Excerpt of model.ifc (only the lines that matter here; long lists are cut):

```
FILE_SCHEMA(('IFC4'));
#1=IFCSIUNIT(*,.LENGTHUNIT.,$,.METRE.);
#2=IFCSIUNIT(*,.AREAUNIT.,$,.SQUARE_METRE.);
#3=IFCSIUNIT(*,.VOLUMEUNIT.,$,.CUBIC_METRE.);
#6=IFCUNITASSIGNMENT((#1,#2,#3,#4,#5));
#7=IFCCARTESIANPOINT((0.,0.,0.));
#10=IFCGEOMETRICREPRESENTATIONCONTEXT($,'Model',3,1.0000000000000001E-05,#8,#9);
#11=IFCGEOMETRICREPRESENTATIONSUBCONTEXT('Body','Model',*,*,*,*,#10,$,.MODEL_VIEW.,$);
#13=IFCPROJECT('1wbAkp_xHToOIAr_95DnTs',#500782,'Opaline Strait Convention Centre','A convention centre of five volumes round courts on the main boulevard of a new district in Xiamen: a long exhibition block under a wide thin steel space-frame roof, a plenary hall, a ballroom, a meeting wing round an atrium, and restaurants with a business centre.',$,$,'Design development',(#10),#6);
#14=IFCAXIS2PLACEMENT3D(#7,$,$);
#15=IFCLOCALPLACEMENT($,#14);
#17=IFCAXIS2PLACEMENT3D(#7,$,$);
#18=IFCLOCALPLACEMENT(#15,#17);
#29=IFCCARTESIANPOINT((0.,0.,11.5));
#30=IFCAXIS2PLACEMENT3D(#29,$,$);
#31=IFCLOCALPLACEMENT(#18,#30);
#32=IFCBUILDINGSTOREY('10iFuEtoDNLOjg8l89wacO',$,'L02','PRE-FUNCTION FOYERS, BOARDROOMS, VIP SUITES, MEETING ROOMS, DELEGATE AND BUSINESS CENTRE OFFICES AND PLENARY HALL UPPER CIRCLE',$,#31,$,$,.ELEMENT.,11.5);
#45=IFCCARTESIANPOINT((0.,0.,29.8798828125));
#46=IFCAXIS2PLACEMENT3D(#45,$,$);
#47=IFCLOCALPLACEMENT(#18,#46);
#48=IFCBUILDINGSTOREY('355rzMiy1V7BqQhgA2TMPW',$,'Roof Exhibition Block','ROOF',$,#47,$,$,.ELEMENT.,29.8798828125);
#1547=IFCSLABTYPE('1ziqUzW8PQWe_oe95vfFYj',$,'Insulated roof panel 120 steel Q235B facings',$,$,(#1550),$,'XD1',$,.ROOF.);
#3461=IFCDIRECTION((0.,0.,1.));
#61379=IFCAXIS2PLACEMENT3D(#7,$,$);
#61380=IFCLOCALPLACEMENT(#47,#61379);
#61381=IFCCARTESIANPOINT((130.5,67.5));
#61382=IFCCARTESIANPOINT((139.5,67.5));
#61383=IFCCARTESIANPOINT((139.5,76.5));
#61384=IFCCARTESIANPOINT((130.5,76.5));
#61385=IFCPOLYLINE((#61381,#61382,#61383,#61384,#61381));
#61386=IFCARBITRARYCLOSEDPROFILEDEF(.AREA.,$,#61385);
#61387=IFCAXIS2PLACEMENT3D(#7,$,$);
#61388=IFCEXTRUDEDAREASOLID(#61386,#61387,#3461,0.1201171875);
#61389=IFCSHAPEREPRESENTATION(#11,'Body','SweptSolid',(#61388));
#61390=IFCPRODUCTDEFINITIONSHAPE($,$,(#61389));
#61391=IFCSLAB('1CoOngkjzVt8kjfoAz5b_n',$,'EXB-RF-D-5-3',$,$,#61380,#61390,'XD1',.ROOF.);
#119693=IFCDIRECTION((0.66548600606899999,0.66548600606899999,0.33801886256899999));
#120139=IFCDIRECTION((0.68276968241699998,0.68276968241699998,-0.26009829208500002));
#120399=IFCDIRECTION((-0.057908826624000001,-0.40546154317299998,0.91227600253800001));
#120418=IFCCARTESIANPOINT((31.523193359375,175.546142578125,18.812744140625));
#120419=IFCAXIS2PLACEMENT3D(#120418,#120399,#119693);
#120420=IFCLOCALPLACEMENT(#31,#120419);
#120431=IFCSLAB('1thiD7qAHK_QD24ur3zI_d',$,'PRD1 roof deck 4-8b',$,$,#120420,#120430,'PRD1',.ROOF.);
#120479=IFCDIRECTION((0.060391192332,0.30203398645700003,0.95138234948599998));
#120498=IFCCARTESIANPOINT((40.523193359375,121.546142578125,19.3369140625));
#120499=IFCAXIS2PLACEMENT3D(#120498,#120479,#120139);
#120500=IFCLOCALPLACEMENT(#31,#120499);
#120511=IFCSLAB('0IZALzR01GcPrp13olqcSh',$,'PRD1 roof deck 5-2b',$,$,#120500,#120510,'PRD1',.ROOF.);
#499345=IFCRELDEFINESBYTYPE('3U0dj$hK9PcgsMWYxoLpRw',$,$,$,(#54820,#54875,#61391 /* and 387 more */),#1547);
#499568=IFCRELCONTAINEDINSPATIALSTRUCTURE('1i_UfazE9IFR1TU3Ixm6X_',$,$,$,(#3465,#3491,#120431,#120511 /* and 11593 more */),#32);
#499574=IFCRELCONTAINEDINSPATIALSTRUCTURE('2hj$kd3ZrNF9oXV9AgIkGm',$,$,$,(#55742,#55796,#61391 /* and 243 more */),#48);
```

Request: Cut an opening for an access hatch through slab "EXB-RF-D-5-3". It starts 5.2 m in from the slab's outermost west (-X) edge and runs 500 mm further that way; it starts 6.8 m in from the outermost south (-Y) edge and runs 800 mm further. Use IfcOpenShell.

```python
import numpy as np
import ifcopenshell
import ifcopenshell.api.feature
import ifcopenshell.api.geometry
import ifcopenshell.api.root
import ifcopenshell.geom
import ifcopenshell.util.placement
import ifcopenshell.util.representation
import ifcopenshell.util.shape
import ifcopenshell.util.unit

model = ifcopenshell.open("model.ifc")
unit_scale = ifcopenshell.util.unit.calculate_unit_scale(model)
settings = ifcopenshell.geom.settings()


def volume(element):
    """Net volume in cubic metres, openings subtracted."""
    shape = ifcopenshell.geom.create_shape(settings, element)
    return ifcopenshell.util.shape.get_volume(shape.geometry)


slab = model.by_guid("1CoOngkjzVt8kjfoAz5b_n")
before = volume(slab)

# Extent in the slab's own axes, in metres. The edges named are its -X and -Y sides.
slab_shape = ifcopenshell.geom.create_shape(settings, slab)
vertices = ifcopenshell.util.shape.get_vertices(slab_shape.geometry)
x_min, y_min, bottom = vertices.min(axis=0)
top = vertices[:, 2].max()

opening = ifcopenshell.api.root.create_entity(model, ifc_class="IfcOpeningElement", name="Access hatch opening", predefined_type="OPENING")
context = ifcopenshell.util.representation.get_context(model, "Model", "Body", "MODEL_VIEW")
width, depth = 0.5, 0.8
outline = [(0.0, 0.0), (width, 0.0), (width, depth), (0.0, depth), (0.0, 0.0)]
# Overshoot both faces by 50 mm so the cut is clean.
shape = ifcopenshell.api.geometry.add_slab_representation(
    model, context=context, depth=top - bottom + 0.1, polyline=outline
)
ifcopenshell.api.geometry.assign_representation(model, product=opening, representation=shape)

matrix = ifcopenshell.util.placement.get_local_placement(slab.ObjectPlacement)
matrix[:, 3] = matrix @ np.append(np.array([x_min + 5.2, y_min + 6.8, bottom - 0.05]) / unit_scale, 1.0)
ifcopenshell.api.geometry.edit_object_placement(model, product=opening, matrix=matrix, is_si=False)
ifcopenshell.api.feature.add_feature(model, feature=opening, element=slab)

after = volume(slab)

print(f"slab volume {before:.3f} -> {after:.3f} m3")

model.write("model_updated.ifc")
```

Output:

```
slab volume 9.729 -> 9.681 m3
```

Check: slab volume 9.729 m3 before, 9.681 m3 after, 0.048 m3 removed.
